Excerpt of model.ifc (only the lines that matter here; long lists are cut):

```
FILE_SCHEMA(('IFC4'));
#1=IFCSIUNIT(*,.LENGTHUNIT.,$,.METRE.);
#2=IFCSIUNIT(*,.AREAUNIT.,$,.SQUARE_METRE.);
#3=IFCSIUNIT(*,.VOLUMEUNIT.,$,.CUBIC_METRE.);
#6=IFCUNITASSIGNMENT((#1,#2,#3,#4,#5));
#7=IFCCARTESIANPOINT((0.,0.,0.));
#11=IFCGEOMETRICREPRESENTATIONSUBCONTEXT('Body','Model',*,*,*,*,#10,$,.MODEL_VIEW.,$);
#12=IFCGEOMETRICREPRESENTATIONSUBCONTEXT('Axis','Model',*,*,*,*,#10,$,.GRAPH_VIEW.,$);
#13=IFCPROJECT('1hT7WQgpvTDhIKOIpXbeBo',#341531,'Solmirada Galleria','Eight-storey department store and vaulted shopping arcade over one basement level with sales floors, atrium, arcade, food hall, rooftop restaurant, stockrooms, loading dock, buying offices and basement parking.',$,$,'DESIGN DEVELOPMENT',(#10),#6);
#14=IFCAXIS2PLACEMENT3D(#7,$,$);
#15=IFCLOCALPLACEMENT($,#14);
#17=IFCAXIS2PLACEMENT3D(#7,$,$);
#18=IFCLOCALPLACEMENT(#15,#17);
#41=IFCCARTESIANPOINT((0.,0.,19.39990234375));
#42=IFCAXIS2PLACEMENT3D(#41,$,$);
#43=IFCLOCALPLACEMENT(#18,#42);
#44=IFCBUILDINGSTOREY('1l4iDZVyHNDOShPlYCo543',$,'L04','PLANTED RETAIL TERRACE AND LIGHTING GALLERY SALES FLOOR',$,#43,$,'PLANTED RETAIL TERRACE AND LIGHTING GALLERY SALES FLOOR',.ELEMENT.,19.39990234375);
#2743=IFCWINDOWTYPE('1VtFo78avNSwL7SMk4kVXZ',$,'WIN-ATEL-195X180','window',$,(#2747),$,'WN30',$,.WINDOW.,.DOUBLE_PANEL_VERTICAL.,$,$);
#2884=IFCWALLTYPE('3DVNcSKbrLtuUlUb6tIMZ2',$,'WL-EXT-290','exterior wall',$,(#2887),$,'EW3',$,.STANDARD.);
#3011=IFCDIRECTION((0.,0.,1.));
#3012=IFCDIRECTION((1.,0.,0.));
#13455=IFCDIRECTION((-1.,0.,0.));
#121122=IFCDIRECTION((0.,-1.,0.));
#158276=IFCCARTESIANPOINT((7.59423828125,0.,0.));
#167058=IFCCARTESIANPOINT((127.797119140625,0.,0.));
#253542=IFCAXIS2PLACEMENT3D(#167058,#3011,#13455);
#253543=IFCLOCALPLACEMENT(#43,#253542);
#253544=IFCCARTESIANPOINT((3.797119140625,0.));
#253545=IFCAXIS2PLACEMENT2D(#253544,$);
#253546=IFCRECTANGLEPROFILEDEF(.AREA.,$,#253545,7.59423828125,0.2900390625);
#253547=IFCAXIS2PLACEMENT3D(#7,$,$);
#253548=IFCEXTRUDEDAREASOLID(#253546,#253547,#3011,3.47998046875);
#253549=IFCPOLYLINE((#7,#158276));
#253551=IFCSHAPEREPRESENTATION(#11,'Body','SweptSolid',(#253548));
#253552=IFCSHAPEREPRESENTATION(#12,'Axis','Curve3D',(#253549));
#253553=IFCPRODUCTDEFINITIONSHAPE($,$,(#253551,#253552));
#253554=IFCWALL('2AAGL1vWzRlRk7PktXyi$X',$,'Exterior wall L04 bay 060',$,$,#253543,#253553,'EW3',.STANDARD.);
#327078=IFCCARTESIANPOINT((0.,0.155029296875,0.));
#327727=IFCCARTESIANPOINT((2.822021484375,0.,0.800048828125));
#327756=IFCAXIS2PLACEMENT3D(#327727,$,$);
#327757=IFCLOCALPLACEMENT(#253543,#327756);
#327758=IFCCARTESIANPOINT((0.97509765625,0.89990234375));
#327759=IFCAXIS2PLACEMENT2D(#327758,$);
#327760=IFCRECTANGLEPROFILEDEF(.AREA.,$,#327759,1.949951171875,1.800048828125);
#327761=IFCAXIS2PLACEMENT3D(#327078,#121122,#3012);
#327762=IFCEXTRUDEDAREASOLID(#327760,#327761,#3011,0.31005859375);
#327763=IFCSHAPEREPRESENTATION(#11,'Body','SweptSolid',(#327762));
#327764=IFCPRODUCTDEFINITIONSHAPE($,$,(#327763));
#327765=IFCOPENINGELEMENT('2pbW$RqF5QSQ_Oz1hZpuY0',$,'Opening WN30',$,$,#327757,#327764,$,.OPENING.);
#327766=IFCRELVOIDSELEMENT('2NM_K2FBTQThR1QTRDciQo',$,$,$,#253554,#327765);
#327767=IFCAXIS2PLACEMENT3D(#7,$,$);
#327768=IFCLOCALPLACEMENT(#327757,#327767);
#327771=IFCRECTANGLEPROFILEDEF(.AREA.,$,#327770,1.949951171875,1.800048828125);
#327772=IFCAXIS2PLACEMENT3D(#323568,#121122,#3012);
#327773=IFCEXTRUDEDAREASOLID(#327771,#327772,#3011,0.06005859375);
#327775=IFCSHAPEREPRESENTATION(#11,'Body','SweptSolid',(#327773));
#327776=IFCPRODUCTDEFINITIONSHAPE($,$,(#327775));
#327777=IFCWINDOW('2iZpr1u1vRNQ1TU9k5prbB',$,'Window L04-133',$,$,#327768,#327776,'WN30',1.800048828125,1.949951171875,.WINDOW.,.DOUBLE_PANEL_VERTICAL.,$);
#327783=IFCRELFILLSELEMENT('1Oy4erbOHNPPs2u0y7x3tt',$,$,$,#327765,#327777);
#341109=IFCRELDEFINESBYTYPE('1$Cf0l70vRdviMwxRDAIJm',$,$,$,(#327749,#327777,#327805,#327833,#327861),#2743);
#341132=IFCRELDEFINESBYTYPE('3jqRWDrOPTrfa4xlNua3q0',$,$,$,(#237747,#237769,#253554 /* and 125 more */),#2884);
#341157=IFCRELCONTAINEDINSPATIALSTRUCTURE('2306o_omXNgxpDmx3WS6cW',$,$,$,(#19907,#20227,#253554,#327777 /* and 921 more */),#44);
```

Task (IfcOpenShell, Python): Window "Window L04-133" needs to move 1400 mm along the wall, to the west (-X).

```python
import ifcopenshell
import ifcopenshell.api.geometry
import ifcopenshell.util.placement

model = ifcopenshell.open("model.ifc")

window = model.by_guid("2iZpr1u1vRNQ1TU9k5prbB")
opening = window.FillsVoids[0].RelatingOpeningElement
wall = opening.VoidsElements[0].RelatingBuildingElement

wall_matrix = ifcopenshell.util.placement.get_local_placement(wall.ObjectPlacement)
shift = wall_matrix[:3, 0] * 1.4
before = ifcopenshell.util.placement.get_local_placement(window.ObjectPlacement)[:3, 3].copy()

# The window is placed relative to its opening, so it follows when the opening moves.
matrix = ifcopenshell.util.placement.get_local_placement(opening.ObjectPlacement)
matrix[:3, 3] += shift
ifcopenshell.api.geometry.edit_object_placement(
    model, product=opening, matrix=matrix, is_si=False, should_transform_children=True
)

after = ifcopenshell.util.placement.get_local_placement(window.ObjectPlacement)[:3, 3]
print("window moved by", (after - before).round(3) + 0.0)

model.write("model_rev.ifc")
```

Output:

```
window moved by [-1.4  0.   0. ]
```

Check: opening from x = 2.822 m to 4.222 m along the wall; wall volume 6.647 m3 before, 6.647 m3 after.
